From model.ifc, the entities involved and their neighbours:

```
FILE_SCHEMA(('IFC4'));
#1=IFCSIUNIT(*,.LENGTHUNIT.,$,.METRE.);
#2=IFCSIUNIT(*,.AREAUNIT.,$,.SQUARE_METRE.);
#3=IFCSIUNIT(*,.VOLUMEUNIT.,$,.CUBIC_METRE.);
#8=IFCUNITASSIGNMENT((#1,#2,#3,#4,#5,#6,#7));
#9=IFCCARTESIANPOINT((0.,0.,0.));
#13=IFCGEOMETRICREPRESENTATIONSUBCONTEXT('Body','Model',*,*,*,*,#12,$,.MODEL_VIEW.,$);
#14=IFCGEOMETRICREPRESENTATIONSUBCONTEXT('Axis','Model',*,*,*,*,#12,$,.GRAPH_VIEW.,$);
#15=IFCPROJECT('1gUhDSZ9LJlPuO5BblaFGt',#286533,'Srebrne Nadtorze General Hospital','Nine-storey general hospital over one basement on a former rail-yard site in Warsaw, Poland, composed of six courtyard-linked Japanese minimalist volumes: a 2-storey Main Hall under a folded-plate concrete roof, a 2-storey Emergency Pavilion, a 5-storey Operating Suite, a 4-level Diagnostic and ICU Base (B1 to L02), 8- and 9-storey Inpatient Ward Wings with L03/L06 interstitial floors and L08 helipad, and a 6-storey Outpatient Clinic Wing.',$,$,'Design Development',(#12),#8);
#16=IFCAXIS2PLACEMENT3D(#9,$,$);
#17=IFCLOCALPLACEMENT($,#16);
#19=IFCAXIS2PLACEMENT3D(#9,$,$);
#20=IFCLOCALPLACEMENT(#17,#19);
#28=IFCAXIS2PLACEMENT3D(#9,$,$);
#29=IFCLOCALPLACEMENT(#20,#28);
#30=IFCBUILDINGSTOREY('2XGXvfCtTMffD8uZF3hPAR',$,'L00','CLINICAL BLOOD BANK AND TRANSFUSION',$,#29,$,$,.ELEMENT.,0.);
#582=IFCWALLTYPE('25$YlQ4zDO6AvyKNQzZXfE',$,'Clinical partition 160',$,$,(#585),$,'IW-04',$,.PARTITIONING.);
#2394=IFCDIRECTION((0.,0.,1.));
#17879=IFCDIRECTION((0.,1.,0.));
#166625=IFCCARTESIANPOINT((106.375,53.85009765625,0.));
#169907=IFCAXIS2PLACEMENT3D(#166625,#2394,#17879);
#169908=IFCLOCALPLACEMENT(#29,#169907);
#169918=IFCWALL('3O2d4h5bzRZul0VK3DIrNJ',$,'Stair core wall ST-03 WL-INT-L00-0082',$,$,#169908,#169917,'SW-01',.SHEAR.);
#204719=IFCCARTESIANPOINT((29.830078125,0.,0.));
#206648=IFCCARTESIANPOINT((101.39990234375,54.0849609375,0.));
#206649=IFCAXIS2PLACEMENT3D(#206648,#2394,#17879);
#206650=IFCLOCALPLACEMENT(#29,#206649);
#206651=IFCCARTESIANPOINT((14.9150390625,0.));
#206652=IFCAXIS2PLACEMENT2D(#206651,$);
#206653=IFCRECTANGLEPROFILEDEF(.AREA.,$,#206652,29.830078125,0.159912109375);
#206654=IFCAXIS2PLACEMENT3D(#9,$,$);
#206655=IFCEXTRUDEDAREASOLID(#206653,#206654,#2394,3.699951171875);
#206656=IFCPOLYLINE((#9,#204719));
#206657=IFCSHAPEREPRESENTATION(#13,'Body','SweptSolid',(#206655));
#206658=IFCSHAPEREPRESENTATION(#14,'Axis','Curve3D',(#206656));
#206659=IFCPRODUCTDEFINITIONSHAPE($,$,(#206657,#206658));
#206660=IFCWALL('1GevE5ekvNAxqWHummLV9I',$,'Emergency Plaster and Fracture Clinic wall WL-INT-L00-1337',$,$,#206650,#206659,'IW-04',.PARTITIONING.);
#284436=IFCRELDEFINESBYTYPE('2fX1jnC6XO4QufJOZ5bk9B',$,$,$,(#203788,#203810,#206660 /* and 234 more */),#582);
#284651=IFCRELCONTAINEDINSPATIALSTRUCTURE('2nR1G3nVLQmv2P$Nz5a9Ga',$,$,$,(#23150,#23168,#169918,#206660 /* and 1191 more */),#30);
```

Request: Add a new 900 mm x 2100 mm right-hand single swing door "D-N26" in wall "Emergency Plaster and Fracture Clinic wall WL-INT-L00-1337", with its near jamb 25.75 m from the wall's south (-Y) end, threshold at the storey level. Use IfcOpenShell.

```python
import numpy as np
import ifcopenshell
import ifcopenshell.api.feature
import ifcopenshell.api.geometry
import ifcopenshell.api.root
import ifcopenshell.api.spatial
import ifcopenshell.geom
import ifcopenshell.util.element
import ifcopenshell.util.placement
import ifcopenshell.util.representation
import ifcopenshell.util.shape
import ifcopenshell.util.unit

model = ifcopenshell.open("model.ifc")
unit_scale = ifcopenshell.util.unit.calculate_unit_scale(model)
settings = ifcopenshell.geom.settings()


def volume(element):
    """Net volume in cubic metres, openings subtracted."""
    shape = ifcopenshell.geom.create_shape(settings, element)
    return ifcopenshell.util.shape.get_volume(shape.geometry)


wall = model.by_guid("1GevE5ekvNAxqWHummLV9I")
storey = ifcopenshell.util.element.get_container(wall, ifc_class="IfcBuildingStorey")
context = ifcopenshell.util.representation.get_context(model, "Model", "Body", "MODEL_VIEW")
before = volume(wall)

width, height, from_end, sill = 0.9, 2.1, 25.75, 0.0  # metres

# The wall runs along its own X axis, and the end named is its -X end.
wall_shape = ifcopenshell.geom.create_shape(settings, wall)
x, y, z = ifcopenshell.util.shape.get_vertices(wall_shape.geometry).T
start = x.min() + from_end
face, thickness = float(y.min()), float(y.max() - y.min())
wall_matrix = ifcopenshell.util.placement.get_local_placement(wall.ObjectPlacement)
level = ifcopenshell.util.placement.get_local_placement(storey.ObjectPlacement)[2, 3]


def in_wall(x, y):
    """Placement at x, y metres in the wall's axes, at sill height."""
    matrix = wall_matrix.copy()
    matrix[:, 3] = wall_matrix @ np.array([x / unit_scale, y / unit_scale, 0.0, 1.0])
    matrix[2, 3] = level + sill / unit_scale
    return matrix


# Opening: a box that overshoots both wall faces by 50 mm.
opening = ifcopenshell.api.root.create_entity(model, ifc_class="IfcOpeningElement", predefined_type="OPENING")
box = ifcopenshell.api.geometry.add_wall_representation(
    model, context=context, length=width, height=height, thickness=thickness + 0.1
)
ifcopenshell.api.geometry.assign_representation(model, product=opening, representation=box)
ifcopenshell.api.geometry.edit_object_placement(model, product=opening, matrix=in_wall(start, face - 0.05), is_si=False)
ifcopenshell.api.feature.add_feature(model, feature=opening, element=wall)

door = ifcopenshell.api.root.create_entity(model, ifc_class="IfcDoor", name="D-N26", predefined_type="DOOR")
door.OverallWidth, door.OverallHeight = width / unit_scale, height / unit_scale
door.OperationType = "SINGLE_SWING_RIGHT"
body = ifcopenshell.api.geometry.add_door_representation(
    model,
    context=context,
    overall_width=door.OverallWidth,
    overall_height=door.OverallHeight,
    operation_type="SINGLE_SWING_RIGHT",
    lining_properties={"LiningDepth": thickness / unit_scale, "ThresholdDepth": thickness / unit_scale},
)
ifcopenshell.api.geometry.assign_representation(model, product=door, representation=body)
ifcopenshell.api.spatial.assign_container(model, products=[door], relating_structure=storey)
ifcopenshell.api.feature.add_filling(model, opening=opening, element=door)

# The lining spans the wall, so the door starts at the wall face.
ifcopenshell.api.geometry.edit_object_placement(model, product=door, matrix=in_wall(start, face), is_si=False)

after = volume(wall)

print(f"wall volume {before:.3f} -> {after:.3f} m3")

model.write("model-out.ifc")
```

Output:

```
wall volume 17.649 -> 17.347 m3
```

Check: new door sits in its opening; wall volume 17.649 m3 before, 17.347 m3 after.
